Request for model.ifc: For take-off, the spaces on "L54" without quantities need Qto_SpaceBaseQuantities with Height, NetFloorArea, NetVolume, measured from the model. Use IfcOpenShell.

First a look at what the model holds.

```python
import ifcopenshell
import ifcopenshell.util.element
import ifcopenshell.util.unit

model = ifcopenshell.open("model.ifc")
print(model.schema)
for unit_type in ("LENGTHUNIT", "AREAUNIT", "VOLUMEUNIT"):
    print(unit_type, ifcopenshell.util.unit.calculate_unit_scale(model, unit_type))
storey = next(s for s in model.by_type("IfcBuildingStorey") if s.Name == "L54")
spaces = [e for e in ifcopenshell.util.element.get_decomposition(storey) if e.is_a("IfcSpace")]
for e in sorted(spaces, key=lambda e: e.id()):
    print(e.id(), e.is_a(), e.Name, list(ifcopenshell.util.element.get_psets(e, qtos_only=True)), sep=" | ")
```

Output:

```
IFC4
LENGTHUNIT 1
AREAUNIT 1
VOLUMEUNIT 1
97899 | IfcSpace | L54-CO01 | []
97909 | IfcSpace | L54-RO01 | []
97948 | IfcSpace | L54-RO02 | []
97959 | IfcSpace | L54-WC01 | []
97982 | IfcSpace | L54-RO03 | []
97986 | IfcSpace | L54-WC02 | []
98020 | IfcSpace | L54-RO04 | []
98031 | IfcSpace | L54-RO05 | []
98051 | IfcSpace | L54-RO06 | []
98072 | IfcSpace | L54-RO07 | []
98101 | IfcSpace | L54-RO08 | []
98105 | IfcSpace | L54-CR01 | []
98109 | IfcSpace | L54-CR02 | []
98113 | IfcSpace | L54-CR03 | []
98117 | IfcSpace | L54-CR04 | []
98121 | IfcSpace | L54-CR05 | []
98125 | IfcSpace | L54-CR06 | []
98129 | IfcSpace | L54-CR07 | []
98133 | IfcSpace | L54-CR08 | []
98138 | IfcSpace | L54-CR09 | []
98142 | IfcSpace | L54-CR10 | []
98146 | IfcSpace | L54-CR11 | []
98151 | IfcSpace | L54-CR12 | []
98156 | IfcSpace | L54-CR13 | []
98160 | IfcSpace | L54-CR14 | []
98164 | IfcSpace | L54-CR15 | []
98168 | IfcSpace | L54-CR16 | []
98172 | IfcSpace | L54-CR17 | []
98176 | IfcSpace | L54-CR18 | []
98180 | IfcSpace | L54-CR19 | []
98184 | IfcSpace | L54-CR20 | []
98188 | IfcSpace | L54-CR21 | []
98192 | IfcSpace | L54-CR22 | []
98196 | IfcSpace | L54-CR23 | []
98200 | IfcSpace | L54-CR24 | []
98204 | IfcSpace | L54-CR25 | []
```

```python
import ifcopenshell
import ifcopenshell.api.pset
import ifcopenshell.geom
import ifcopenshell.util.element
import ifcopenshell.util.shape
import ifcopenshell.util.unit

model = ifcopenshell.open("model.ifc")
unit_scale = ifcopenshell.util.unit.calculate_unit_scale(model)
area_scale = ifcopenshell.util.unit.calculate_unit_scale(model, "AREAUNIT")
volume_scale = ifcopenshell.util.unit.calculate_unit_scale(model, "VOLUMEUNIT")
settings = ifcopenshell.geom.settings()

storey = next(s for s in model.by_type("IfcBuildingStorey") if s.Name == "L54")
spaces = [e for e in ifcopenshell.util.element.get_decomposition(storey) if e.is_a("IfcSpace")]

for e in sorted(spaces, key=lambda e: e.id()):
    if ifcopenshell.util.element.get_psets(e, qtos_only=True, should_inherit=False):
        continue
    # Geometry comes back in metres, in the element's own axes.
    shape = ifcopenshell.geom.create_shape(settings, e)
    values = {
        "Height": ifcopenshell.util.shape.get_z(shape.geometry) / unit_scale,
        "NetFloorArea": ifcopenshell.util.shape.get_footprint_area(shape.geometry) / area_scale,
        "NetVolume": ifcopenshell.util.shape.get_volume(shape.geometry) / volume_scale,
    }
    qto = ifcopenshell.api.pset.add_qto(model, product=e, name="Qto_SpaceBaseQuantities")
    ifcopenshell.api.pset.edit_qto(model, qto=qto, properties=values)
    print(e.id(), {k: round(v, 3) for k, v in values.items()})

model.write("model_edited.ifc")
```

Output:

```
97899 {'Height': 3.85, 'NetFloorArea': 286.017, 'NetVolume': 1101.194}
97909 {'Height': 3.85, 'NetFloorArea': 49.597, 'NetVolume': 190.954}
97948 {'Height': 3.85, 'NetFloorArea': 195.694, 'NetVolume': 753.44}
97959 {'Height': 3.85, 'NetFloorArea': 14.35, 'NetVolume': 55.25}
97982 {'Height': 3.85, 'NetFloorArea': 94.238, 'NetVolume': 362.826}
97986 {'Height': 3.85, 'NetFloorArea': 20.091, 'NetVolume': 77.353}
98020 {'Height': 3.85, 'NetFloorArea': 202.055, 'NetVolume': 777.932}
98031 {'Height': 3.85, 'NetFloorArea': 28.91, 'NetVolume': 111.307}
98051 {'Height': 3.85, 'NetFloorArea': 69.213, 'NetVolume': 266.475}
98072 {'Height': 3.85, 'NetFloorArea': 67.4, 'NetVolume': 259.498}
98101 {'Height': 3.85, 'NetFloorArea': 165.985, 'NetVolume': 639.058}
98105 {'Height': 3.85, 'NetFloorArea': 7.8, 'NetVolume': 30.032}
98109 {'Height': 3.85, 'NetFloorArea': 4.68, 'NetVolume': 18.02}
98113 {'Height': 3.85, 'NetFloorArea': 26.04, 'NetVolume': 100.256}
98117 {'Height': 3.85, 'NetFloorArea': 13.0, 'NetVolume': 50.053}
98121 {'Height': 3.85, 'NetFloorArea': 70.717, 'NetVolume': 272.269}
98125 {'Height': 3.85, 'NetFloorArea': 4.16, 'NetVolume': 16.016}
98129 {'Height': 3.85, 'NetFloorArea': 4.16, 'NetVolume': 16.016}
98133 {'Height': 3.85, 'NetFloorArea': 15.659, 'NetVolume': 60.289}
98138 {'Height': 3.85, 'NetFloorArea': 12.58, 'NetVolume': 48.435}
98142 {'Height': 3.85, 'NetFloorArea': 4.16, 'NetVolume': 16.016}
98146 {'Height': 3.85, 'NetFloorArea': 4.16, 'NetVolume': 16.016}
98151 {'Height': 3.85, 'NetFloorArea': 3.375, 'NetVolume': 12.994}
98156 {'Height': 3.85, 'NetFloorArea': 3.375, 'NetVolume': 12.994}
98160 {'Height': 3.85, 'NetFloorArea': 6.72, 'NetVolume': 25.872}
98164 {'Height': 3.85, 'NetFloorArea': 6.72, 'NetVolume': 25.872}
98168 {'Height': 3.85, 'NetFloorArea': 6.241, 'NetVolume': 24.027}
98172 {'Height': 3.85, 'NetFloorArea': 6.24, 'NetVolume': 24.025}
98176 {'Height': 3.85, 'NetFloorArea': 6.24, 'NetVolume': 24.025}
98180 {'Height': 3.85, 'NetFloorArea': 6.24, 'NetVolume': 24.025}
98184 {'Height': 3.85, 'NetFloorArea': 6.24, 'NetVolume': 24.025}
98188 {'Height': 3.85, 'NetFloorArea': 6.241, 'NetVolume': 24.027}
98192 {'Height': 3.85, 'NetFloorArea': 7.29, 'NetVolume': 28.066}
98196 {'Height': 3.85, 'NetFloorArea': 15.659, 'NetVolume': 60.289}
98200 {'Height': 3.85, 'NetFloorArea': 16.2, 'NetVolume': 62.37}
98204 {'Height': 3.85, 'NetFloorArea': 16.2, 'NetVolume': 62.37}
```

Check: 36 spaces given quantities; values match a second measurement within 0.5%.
